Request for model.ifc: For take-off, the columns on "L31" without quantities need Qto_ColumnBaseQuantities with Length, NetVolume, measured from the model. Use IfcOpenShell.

First a look at what the model holds.

```python
import ifcopenshell
import ifcopenshell.util.element
import ifcopenshell.util.unit

model = ifcopenshell.open("model.ifc")
print(model.schema)
for unit_type in ("LENGTHUNIT", "AREAUNIT", "VOLUMEUNIT"):
    print(unit_type, ifcopenshell.util.unit.calculate_unit_scale(model, unit_type))
storey = next(s for s in model.by_type("IfcBuildingStorey") if s.Name == "L31")
columns = [e for e in ifcopenshell.util.element.get_decomposition(storey) if e.is_a("IfcColumn")]
for e in sorted(columns, key=lambda e: e.id()):
    print(e.id(), e.is_a(), e.Name, list(ifcopenshell.util.element.get_psets(e, qtos_only=True)), sep=" | ")
```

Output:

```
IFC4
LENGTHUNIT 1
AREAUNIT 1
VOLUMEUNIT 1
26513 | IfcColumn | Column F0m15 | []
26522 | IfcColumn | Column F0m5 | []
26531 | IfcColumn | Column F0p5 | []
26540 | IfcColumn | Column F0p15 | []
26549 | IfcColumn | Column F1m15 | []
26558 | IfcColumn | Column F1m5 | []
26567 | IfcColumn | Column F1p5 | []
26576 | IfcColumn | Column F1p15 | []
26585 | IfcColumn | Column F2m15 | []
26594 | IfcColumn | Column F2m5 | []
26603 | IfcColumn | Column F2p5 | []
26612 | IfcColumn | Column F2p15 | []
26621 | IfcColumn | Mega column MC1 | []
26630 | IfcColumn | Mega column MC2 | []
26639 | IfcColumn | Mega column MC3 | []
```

```python
import ifcopenshell
import ifcopenshell.api.pset
import ifcopenshell.geom
import ifcopenshell.util.element
import ifcopenshell.util.shape
import ifcopenshell.util.unit

model = ifcopenshell.open("model.ifc")
unit_scale = ifcopenshell.util.unit.calculate_unit_scale(model)
volume_scale = ifcopenshell.util.unit.calculate_unit_scale(model, "VOLUMEUNIT")
settings = ifcopenshell.geom.settings()

storey = next(s for s in model.by_type("IfcBuildingStorey") if s.Name == "L31")
columns = [e for e in ifcopenshell.util.element.get_decomposition(storey) if e.is_a("IfcColumn")]

for e in sorted(columns, key=lambda e: e.id()):
    if ifcopenshell.util.element.get_psets(e, qtos_only=True, should_inherit=False):
        continue
    # Geometry comes back in metres, in the element's own axes.
    shape = ifcopenshell.geom.create_shape(settings, e)
    values = {
        "Length": ifcopenshell.util.shape.get_z(shape.geometry) / unit_scale,
        "NetVolume": ifcopenshell.util.shape.get_volume(shape.geometry) / volume_scale,
    }
    qto = ifcopenshell.api.pset.add_qto(model, product=e, name="Qto_ColumnBaseQuantities")
    ifcopenshell.api.pset.edit_qto(model, qto=qto, properties=values)
    print(e.id(), {k: round(v, 3) for k, v in values.items()})

model.write("model_v2.ifc")
```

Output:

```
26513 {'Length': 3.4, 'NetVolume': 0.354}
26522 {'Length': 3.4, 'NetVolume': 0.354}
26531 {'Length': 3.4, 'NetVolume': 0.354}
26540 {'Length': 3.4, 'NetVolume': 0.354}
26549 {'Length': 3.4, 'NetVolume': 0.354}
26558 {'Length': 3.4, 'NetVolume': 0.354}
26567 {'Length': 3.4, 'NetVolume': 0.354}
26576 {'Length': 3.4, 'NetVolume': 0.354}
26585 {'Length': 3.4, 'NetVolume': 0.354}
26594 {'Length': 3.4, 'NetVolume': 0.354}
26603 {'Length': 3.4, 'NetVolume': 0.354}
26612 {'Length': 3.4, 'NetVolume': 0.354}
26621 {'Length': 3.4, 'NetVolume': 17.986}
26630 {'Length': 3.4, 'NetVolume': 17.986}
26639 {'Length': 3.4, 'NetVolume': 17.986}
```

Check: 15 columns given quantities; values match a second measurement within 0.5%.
